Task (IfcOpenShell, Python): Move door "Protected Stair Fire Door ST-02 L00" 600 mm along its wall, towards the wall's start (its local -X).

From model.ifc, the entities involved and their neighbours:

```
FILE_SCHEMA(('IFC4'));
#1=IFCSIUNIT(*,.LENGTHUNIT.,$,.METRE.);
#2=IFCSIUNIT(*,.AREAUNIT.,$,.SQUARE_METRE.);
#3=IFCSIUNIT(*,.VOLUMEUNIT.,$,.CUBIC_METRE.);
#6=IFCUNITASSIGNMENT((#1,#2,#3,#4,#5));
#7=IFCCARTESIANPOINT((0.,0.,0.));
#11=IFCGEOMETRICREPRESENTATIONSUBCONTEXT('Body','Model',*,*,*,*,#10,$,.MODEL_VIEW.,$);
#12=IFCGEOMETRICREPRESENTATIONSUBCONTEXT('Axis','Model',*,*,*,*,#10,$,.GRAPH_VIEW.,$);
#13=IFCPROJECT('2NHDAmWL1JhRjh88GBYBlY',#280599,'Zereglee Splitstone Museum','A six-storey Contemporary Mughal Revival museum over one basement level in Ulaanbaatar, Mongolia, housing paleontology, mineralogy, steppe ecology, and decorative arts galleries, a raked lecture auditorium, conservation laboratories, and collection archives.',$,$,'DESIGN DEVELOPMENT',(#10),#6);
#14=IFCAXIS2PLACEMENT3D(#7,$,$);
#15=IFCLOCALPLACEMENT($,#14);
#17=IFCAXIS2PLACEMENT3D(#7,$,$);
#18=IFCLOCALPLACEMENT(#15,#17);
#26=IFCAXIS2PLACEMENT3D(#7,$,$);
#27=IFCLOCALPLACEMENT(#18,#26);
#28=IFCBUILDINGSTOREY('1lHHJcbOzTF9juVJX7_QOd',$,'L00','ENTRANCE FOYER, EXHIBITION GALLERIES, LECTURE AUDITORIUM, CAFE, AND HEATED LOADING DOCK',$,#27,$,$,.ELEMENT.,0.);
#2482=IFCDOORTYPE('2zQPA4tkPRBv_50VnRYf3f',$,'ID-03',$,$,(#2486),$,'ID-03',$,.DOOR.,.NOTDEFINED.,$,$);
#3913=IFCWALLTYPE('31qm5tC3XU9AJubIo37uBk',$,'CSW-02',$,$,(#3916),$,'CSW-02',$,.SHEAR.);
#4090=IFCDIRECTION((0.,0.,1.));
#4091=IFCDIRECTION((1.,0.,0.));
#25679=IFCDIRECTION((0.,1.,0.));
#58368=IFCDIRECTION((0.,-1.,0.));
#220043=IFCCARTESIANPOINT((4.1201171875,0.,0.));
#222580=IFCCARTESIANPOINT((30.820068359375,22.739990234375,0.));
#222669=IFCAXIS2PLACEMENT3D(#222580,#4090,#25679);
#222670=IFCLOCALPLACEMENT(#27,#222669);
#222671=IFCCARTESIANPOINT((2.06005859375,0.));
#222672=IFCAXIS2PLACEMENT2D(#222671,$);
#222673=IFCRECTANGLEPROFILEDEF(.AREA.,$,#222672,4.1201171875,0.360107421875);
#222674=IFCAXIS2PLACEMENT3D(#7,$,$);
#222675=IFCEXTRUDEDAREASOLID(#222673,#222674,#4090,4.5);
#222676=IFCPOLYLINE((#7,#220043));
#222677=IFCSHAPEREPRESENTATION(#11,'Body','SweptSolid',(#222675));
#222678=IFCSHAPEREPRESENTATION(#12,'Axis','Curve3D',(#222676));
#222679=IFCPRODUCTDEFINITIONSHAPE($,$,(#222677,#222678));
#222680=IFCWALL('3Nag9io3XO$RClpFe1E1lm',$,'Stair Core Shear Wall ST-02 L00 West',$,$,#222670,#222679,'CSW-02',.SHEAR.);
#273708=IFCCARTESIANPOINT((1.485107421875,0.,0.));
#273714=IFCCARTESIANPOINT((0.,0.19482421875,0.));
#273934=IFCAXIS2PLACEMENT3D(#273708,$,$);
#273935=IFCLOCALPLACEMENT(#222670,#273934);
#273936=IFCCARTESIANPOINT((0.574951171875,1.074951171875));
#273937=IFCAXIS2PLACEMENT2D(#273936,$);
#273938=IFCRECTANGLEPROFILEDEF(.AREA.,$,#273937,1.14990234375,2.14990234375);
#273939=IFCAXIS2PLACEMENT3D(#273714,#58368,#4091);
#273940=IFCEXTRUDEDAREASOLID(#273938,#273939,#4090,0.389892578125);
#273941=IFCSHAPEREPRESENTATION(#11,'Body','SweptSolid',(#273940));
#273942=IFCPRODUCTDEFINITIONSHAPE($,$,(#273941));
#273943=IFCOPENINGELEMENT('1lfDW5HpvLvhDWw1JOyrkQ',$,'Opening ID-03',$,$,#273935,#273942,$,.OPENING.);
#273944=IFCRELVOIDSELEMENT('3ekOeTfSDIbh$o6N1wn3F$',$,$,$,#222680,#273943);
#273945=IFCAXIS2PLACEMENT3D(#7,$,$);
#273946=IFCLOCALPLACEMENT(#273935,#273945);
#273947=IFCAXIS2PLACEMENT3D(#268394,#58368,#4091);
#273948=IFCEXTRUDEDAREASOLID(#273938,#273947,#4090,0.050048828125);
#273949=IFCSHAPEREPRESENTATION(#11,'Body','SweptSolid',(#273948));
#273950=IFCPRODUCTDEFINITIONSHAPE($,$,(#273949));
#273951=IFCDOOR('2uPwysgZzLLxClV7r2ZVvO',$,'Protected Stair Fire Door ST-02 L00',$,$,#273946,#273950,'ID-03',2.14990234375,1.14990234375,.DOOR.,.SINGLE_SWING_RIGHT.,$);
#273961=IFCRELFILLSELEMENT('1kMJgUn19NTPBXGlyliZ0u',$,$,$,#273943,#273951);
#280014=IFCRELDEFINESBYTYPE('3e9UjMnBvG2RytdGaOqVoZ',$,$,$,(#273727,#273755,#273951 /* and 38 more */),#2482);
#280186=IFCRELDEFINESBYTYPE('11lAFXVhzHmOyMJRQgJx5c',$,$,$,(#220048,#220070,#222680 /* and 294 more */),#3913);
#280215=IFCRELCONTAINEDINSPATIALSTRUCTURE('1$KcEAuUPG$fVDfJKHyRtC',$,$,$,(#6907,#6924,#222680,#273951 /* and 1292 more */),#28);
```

```python
import ifcopenshell
import ifcopenshell.api.geometry
import ifcopenshell.util.placement
import ifcopenshell.util.unit

model = ifcopenshell.open("model.ifc")
unit_scale = ifcopenshell.util.unit.calculate_unit_scale(model)

door = model.by_guid("2uPwysgZzLLxClV7r2ZVvO")
opening = door.FillsVoids[0].RelatingOpeningElement
wall = opening.VoidsElements[0].RelatingBuildingElement

wall_matrix = ifcopenshell.util.placement.get_local_placement(wall.ObjectPlacement)
shift = wall_matrix[:3, 0] * -0.6 / unit_scale
before = ifcopenshell.util.placement.get_local_placement(door.ObjectPlacement)[:3, 3].copy()

# The door is placed relative to its opening, so it follows when the opening moves.
matrix = ifcopenshell.util.placement.get_local_placement(opening.ObjectPlacement)
matrix[:3, 3] += shift
ifcopenshell.api.geometry.edit_object_placement(
    model, product=opening, matrix=matrix, is_si=False, should_transform_children=True
)

after = ifcopenshell.util.placement.get_local_placement(door.ObjectPlacement)[:3, 3]
print("door moved by", (after - before).round(3) + 0.0)

model.write("model_rev.ifc")
```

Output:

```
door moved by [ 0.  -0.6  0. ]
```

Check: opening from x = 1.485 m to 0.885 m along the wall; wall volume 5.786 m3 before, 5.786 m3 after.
